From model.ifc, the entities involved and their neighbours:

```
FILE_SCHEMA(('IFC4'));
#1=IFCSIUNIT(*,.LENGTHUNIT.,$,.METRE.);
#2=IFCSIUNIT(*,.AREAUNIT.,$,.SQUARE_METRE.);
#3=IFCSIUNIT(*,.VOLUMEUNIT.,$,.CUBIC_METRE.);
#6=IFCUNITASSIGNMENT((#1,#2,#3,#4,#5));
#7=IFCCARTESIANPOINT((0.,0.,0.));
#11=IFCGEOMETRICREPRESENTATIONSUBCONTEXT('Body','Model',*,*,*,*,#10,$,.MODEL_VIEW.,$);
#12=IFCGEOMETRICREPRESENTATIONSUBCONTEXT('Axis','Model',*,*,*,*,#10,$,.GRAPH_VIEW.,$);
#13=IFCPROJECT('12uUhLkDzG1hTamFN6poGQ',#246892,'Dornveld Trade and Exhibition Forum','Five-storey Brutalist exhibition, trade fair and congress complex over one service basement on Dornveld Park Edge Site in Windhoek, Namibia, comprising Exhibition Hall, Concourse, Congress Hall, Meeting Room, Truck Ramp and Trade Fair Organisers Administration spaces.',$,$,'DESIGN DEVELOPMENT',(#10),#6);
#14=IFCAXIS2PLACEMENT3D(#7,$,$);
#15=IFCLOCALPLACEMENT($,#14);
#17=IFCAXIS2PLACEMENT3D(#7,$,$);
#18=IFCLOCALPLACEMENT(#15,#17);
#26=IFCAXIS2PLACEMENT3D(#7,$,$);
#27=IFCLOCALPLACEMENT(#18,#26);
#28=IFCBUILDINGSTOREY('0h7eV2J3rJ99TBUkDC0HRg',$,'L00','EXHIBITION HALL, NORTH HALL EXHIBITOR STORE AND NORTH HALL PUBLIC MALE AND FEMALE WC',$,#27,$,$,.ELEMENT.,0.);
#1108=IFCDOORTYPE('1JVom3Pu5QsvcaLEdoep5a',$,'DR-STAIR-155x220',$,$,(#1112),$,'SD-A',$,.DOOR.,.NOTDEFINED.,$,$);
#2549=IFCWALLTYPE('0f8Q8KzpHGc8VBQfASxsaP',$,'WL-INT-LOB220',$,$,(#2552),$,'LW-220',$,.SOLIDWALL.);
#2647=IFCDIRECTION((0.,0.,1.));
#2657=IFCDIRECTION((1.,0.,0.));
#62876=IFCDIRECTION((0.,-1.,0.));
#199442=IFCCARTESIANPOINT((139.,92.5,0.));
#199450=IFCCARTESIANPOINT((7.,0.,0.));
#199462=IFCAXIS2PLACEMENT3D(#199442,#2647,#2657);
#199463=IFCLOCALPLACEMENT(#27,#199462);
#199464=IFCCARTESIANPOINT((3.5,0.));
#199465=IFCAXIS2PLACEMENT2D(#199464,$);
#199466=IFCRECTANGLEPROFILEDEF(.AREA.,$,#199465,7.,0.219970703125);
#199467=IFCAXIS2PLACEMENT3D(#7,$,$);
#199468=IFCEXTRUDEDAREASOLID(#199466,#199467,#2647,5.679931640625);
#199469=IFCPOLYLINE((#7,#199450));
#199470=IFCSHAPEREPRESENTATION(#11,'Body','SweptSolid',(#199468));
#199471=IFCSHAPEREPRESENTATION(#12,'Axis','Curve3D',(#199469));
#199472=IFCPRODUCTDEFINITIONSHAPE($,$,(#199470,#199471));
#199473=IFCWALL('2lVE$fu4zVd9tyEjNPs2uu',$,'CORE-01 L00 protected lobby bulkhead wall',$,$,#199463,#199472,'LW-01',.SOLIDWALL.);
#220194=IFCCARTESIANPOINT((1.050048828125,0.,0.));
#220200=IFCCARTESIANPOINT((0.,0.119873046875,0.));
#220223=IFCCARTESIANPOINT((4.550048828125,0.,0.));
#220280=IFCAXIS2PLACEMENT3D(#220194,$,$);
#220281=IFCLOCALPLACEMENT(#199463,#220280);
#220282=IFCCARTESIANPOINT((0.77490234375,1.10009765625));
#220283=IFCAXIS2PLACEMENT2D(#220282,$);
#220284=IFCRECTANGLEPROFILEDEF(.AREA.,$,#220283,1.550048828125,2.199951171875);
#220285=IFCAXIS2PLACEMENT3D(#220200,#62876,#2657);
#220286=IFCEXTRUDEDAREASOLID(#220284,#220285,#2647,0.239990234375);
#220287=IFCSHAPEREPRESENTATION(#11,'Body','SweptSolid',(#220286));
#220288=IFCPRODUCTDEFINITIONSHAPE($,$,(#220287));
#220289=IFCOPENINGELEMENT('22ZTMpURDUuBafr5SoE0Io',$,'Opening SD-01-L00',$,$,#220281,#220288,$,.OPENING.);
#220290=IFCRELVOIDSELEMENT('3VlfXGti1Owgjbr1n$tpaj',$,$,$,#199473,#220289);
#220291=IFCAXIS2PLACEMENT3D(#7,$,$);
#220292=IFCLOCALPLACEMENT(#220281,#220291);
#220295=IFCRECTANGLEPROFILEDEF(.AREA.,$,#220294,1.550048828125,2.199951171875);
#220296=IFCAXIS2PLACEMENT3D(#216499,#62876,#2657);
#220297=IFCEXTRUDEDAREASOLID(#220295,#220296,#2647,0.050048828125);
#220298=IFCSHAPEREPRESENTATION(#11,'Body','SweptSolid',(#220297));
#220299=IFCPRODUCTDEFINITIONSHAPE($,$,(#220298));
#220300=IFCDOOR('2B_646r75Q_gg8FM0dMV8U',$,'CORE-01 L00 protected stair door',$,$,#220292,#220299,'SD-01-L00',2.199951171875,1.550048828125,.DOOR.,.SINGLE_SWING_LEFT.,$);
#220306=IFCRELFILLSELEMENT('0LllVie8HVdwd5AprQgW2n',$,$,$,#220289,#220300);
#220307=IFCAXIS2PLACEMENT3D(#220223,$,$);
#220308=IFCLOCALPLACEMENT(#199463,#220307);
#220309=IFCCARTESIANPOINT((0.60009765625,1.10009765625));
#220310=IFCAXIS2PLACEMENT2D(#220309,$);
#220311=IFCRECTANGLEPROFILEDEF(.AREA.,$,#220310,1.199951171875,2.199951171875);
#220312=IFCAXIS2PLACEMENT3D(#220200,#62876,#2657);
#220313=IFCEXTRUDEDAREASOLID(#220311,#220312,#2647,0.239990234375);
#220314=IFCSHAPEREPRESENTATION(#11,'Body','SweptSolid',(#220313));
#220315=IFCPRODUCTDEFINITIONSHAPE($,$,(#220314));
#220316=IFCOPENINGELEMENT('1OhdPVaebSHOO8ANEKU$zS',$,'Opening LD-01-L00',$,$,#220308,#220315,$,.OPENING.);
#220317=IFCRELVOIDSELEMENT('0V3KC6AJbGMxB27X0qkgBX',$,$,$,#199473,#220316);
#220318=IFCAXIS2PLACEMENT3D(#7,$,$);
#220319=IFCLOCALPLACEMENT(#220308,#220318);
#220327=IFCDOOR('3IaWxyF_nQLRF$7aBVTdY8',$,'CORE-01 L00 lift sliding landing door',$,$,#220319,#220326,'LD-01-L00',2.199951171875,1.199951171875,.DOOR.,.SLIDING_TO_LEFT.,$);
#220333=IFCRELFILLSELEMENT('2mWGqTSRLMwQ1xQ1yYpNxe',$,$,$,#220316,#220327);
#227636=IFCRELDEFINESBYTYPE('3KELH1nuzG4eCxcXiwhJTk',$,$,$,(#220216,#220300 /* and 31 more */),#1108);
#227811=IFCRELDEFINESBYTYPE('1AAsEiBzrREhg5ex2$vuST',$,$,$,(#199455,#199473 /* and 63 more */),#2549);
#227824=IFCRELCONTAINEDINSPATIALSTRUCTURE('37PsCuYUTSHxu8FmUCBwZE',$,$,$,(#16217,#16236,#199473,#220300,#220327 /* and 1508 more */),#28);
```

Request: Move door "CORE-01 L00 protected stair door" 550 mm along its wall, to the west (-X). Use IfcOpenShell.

```python
import ifcopenshell
import ifcopenshell.api.geometry
import ifcopenshell.util.placement
import ifcopenshell.util.unit

model = ifcopenshell.open("model.ifc")
unit_scale = ifcopenshell.util.unit.calculate_unit_scale(model)

door = model.by_id(220300)
opening = door.FillsVoids[0].RelatingOpeningElement
wall = opening.VoidsElements[0].RelatingBuildingElement

wall_matrix = ifcopenshell.util.placement.get_local_placement(wall.ObjectPlacement)
shift = wall_matrix[:3, 0] * -0.55 / unit_scale
before = ifcopenshell.util.placement.get_local_placement(door.ObjectPlacement)[:3, 3].copy()

# The door is placed relative to its opening, so it follows when the opening moves.
matrix = ifcopenshell.util.placement.get_local_placement(opening.ObjectPlacement)
matrix[:3, 3] += shift
ifcopenshell.api.geometry.edit_object_placement(
    model, product=opening, matrix=matrix, is_si=False, should_transform_children=True
)

after = ifcopenshell.util.placement.get_local_placement(door.ObjectPlacement)[:3, 3]
print("door moved by", (after - before).round(3) + 0.0)

model.write("model_edited.ifc")
```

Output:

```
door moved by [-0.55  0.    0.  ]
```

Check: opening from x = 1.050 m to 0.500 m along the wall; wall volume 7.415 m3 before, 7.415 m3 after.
